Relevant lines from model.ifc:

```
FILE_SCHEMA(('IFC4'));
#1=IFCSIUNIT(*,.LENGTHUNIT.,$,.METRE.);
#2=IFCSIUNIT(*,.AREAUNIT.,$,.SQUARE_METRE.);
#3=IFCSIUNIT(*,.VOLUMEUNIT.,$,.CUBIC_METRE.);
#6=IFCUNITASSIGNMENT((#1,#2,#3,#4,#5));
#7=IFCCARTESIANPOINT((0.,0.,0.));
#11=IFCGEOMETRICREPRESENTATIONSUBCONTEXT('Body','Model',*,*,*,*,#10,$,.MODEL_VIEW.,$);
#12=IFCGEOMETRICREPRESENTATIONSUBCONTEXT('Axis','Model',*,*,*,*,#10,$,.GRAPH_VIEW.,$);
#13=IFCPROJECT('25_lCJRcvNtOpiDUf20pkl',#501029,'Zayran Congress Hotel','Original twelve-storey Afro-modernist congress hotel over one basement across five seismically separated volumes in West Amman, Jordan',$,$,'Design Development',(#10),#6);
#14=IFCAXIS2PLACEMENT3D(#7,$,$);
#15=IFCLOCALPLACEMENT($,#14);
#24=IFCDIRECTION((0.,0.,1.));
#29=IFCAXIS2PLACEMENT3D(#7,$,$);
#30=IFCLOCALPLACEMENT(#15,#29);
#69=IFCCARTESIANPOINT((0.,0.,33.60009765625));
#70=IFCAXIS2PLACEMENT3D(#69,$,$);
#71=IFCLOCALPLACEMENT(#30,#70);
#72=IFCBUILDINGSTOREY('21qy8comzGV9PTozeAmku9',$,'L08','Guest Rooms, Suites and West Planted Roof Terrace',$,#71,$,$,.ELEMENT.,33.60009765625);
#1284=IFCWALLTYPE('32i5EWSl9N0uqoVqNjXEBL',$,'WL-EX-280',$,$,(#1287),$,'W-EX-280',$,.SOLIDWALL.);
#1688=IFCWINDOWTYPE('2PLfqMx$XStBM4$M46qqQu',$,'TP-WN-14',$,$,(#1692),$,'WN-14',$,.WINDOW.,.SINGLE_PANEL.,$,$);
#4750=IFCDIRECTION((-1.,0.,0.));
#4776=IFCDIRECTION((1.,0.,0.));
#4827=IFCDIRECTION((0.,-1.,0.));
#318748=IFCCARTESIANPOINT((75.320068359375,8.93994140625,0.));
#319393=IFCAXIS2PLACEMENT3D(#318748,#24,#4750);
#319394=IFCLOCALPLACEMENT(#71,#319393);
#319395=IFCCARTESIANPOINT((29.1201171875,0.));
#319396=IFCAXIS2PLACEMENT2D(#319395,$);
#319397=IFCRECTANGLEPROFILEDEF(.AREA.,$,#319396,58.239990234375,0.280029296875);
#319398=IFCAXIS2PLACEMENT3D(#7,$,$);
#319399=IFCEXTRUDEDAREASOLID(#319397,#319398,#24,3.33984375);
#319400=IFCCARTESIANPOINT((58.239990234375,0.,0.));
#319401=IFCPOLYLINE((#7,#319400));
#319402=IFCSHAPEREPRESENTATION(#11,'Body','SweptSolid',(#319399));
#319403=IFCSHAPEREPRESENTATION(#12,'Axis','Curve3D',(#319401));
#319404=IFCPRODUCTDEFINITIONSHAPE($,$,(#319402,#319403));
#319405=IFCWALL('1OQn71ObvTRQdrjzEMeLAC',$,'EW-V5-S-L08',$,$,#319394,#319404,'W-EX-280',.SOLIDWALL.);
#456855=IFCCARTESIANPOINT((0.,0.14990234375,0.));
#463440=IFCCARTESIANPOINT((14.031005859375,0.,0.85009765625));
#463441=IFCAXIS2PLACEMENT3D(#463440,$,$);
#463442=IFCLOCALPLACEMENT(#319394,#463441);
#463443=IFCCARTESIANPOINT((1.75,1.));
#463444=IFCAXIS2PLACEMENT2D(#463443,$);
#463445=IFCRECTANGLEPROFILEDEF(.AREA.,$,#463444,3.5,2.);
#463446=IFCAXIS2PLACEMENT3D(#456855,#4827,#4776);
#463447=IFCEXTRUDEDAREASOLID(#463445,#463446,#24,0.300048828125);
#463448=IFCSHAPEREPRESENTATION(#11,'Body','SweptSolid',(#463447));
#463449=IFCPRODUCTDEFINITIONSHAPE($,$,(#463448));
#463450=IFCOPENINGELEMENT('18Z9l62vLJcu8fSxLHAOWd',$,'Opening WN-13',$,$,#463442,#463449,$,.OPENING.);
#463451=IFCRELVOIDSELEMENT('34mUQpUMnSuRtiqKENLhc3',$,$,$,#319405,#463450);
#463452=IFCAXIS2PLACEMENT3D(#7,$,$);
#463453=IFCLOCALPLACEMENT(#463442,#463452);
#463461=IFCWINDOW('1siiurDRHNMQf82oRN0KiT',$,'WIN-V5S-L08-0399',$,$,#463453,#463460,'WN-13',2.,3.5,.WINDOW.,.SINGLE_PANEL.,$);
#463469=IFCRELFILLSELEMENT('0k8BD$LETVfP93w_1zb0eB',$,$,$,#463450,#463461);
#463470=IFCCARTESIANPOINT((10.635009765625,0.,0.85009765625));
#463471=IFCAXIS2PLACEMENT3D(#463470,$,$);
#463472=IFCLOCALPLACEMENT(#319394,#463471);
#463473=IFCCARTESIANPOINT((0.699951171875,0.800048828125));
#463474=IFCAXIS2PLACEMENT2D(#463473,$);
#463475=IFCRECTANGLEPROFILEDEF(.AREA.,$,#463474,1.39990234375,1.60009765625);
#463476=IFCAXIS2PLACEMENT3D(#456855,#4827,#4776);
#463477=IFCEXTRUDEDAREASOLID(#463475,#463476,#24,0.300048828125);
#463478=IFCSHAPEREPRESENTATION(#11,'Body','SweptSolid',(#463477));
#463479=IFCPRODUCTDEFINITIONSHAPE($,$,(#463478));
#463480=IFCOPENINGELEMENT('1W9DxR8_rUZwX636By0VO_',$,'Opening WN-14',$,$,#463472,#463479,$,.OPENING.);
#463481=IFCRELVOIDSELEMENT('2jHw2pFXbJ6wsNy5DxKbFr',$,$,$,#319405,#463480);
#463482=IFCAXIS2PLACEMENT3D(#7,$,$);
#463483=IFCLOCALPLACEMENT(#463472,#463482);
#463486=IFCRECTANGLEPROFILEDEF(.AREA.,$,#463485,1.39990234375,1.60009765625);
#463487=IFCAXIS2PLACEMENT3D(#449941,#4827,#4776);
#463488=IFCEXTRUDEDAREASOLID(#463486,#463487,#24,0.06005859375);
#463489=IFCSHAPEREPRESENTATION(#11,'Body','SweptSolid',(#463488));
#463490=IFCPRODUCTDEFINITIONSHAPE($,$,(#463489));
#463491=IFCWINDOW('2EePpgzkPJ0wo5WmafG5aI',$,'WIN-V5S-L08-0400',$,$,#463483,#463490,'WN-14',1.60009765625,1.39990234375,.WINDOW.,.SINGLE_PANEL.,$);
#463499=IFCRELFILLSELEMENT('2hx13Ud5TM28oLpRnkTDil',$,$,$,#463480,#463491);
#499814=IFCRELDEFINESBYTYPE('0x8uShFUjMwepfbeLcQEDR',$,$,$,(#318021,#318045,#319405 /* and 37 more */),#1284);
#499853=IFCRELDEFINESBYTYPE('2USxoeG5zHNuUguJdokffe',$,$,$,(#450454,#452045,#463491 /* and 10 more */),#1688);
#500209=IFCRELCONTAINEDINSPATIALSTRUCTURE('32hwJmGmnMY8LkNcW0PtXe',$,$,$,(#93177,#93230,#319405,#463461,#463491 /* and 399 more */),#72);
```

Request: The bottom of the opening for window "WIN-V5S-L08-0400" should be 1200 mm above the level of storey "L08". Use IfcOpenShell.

```python
import numpy as np
import ifcopenshell
import ifcopenshell.api.geometry
import ifcopenshell.geom
import ifcopenshell.util.element
import ifcopenshell.util.placement
import ifcopenshell.util.shape
import ifcopenshell.util.unit

model = ifcopenshell.open("model.ifc")
unit_scale = ifcopenshell.util.unit.calculate_unit_scale(model)

window = model.by_guid("2EePpgzkPJ0wo5WmafG5aI")
opening = window.FillsVoids[0].RelatingOpeningElement
storey = ifcopenshell.util.element.get_container(window, ifc_class="IfcBuildingStorey")
level = ifcopenshell.util.placement.get_local_placement(storey.ObjectPlacement)[2, 3]

# The opening's origin need not be at the sill, so measure its lowest point.
shape = ifcopenshell.geom.create_shape(ifcopenshell.geom.settings(), opening)
bottom = ifcopenshell.util.shape.get_shape_bottom_elevation(shape, shape.geometry) / unit_scale
dz = level + 1.2 - bottom

shift = np.array([0.0, 0.0, dz])
# The window is placed relative to its opening, so it follows when the opening moves.
matrix = ifcopenshell.util.placement.get_local_placement(opening.ObjectPlacement)
matrix[:3, 3] += shift
ifcopenshell.api.geometry.edit_object_placement(
    model, product=opening, matrix=matrix, is_si=False, should_transform_children=True
)

print(f"moved by {dz * unit_scale:+.3f} m")

model.write("model-out.ifc")
```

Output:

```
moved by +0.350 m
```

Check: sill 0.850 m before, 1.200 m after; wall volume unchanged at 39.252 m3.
